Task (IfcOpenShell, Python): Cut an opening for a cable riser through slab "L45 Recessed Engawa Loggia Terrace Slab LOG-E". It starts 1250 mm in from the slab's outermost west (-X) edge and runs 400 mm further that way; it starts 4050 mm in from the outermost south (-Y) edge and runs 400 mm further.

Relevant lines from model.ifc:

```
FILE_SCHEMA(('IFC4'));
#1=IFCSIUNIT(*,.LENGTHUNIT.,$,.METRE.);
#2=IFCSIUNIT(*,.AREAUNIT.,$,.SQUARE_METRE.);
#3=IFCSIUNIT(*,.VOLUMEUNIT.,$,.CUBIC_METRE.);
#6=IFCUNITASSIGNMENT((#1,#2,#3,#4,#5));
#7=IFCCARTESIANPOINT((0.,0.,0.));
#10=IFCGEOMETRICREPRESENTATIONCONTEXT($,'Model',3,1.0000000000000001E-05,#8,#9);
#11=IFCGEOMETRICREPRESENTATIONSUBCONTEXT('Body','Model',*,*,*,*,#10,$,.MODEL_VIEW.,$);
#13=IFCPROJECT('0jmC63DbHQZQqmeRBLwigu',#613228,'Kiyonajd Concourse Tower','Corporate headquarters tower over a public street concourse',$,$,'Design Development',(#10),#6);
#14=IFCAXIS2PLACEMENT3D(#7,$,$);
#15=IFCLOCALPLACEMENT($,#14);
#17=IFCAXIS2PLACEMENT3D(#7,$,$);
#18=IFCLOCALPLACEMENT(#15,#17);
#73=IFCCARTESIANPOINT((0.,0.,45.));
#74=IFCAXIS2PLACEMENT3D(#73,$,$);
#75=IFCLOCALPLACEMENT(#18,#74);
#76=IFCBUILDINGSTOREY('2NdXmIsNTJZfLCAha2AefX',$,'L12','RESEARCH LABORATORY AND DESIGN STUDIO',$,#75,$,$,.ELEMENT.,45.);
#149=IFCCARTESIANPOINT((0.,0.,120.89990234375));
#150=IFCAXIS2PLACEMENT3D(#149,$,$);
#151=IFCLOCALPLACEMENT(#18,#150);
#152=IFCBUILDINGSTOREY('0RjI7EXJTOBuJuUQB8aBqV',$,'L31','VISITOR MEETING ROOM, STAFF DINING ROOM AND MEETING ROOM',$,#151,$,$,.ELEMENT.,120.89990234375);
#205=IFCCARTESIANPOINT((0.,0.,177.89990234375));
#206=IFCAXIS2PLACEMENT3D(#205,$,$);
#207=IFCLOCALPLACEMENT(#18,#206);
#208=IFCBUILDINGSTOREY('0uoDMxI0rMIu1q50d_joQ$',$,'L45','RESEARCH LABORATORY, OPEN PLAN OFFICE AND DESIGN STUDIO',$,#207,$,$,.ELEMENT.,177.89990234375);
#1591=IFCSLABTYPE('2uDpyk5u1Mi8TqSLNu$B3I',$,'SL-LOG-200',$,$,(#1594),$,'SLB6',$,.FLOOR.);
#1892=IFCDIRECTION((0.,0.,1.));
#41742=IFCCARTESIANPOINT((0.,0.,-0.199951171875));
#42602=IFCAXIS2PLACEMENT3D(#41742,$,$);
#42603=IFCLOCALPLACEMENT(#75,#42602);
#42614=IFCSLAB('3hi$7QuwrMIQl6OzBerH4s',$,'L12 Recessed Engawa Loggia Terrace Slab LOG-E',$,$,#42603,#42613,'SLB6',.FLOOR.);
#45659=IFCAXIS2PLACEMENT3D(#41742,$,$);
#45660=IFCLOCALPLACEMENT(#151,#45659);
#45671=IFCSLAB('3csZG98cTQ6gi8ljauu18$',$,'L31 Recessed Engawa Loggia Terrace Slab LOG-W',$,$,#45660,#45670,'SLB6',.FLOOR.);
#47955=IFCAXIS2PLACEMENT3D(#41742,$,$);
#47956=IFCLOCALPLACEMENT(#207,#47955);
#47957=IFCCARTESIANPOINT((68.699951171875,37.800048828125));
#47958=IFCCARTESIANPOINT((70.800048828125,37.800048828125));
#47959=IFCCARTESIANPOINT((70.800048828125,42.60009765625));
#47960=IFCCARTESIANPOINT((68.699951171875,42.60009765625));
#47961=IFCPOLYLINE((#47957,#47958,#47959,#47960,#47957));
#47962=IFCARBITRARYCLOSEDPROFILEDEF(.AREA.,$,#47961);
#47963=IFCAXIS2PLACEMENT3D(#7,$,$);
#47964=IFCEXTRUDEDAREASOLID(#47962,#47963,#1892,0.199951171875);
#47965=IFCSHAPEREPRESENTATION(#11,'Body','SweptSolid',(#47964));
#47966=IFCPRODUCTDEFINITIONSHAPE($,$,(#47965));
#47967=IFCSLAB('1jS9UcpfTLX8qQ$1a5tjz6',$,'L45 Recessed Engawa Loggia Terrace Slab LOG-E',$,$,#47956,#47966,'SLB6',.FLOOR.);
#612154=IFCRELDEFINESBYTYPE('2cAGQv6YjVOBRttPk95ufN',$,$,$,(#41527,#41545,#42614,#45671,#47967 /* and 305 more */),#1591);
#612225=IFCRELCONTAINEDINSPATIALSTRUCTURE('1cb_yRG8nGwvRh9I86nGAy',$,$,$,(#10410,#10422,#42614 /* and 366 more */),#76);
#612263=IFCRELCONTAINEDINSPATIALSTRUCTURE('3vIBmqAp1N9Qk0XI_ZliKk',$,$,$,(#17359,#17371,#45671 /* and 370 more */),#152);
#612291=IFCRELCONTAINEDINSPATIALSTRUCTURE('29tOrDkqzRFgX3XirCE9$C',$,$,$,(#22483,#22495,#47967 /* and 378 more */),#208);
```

```python
import numpy as np
import ifcopenshell
import ifcopenshell.api.feature
import ifcopenshell.api.geometry
import ifcopenshell.api.root
import ifcopenshell.geom
import ifcopenshell.util.placement
import ifcopenshell.util.representation
import ifcopenshell.util.shape
import ifcopenshell.util.unit

model = ifcopenshell.open("model.ifc")
unit_scale = ifcopenshell.util.unit.calculate_unit_scale(model)
settings = ifcopenshell.geom.settings()


def volume(element):
    """Net volume in cubic metres, openings subtracted."""
    shape = ifcopenshell.geom.create_shape(settings, element)
    return ifcopenshell.util.shape.get_volume(shape.geometry)


slab = model.by_id(47967)
before = volume(slab)

# Extent in the slab's own axes, in metres. The edges named are its -X and -Y sides.
slab_shape = ifcopenshell.geom.create_shape(settings, slab)
vertices = ifcopenshell.util.shape.get_vertices(slab_shape.geometry)
x_min, y_min, bottom = vertices.min(axis=0)
top = vertices[:, 2].max()

opening = ifcopenshell.api.root.create_entity(model, ifc_class="IfcOpeningElement", name="Cable riser opening", predefined_type="OPENING")
context = ifcopenshell.util.representation.get_context(model, "Model", "Body", "MODEL_VIEW")
width, depth = 0.4, 0.4
outline = [(0.0, 0.0), (width, 0.0), (width, depth), (0.0, depth), (0.0, 0.0)]
# Overshoot both faces by 50 mm so the cut is clean.
shape = ifcopenshell.api.geometry.add_slab_representation(
    model, context=context, depth=top - bottom + 0.1, polyline=outline
)
ifcopenshell.api.geometry.assign_representation(model, product=opening, representation=shape)

matrix = ifcopenshell.util.placement.get_local_placement(slab.ObjectPlacement)
matrix[:, 3] = matrix @ np.append(np.array([x_min + 1.25, y_min + 4.05, bottom - 0.05]) / unit_scale, 1.0)
ifcopenshell.api.geometry.edit_object_placement(model, product=opening, matrix=matrix, is_si=False)
ifcopenshell.api.feature.add_feature(model, feature=opening, element=slab)

after = volume(slab)

print(f"slab volume {before:.3f} -> {after:.3f} m3")

model.write("model-out.ifc")
```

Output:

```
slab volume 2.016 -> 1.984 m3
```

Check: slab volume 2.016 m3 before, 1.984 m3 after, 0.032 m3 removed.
